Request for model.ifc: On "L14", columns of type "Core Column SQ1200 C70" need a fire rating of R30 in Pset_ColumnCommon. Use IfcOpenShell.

First a look at what the model holds.

```python
import ifcopenshell
import ifcopenshell.util.element

model = ifcopenshell.open("model.ifc")
print(model.schema)
storey = next(s for s in model.by_type("IfcBuildingStorey") if s.Name == "L14")
columns = [e for e in ifcopenshell.util.element.get_decomposition(storey) if e.is_a("IfcColumn")]
seen = {}
for e in columns:
    element_type = ifcopenshell.util.element.get_type(e)
    key = (element_type.Name if element_type != e and element_type else None, ifcopenshell.util.element.get_pset(e, "Pset_ColumnCommon", "FireRating"))
    seen[key] = seen.get(key, 0) + 1
for (name, value), count in sorted(seen.items(), key=str):
    print(count, "x", name, "|", value)
```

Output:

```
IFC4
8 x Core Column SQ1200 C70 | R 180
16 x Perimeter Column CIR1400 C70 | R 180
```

```python
import ifcopenshell
import ifcopenshell.api.pset
import ifcopenshell.util.element

model = ifcopenshell.open("model.ifc")

storey = next(s for s in model.by_type("IfcBuildingStorey") if s.Name == "L14")
columns = [e for e in ifcopenshell.util.element.get_decomposition(storey) if e.is_a("IfcColumn")]

count = 0
for e in columns:
    element_type = ifcopenshell.util.element.get_type(e)
    if element_type in (None, e) or element_type.Name != "Core Column SQ1200 C70":
        continue
    found = ifcopenshell.util.element.get_pset(e, "Pset_ColumnCommon", should_inherit=False)
    if found:
        pset = model.by_id(found["id"])
        if len(ifcopenshell.util.element.get_elements_by_pset(pset)) > 1:
            pset = ifcopenshell.api.pset.unshare_pset(model, products=[e], pset=pset)[0]
    else:
        pset = ifcopenshell.api.pset.add_pset(model, product=e, name="Pset_ColumnCommon")
    ifcopenshell.api.pset.edit_pset(model, pset=pset, properties={"FireRating": "R30"})
    count += 1

print(count, "columns updated")

model.write("model_v2.ifc")
```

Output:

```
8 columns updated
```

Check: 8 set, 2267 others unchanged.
